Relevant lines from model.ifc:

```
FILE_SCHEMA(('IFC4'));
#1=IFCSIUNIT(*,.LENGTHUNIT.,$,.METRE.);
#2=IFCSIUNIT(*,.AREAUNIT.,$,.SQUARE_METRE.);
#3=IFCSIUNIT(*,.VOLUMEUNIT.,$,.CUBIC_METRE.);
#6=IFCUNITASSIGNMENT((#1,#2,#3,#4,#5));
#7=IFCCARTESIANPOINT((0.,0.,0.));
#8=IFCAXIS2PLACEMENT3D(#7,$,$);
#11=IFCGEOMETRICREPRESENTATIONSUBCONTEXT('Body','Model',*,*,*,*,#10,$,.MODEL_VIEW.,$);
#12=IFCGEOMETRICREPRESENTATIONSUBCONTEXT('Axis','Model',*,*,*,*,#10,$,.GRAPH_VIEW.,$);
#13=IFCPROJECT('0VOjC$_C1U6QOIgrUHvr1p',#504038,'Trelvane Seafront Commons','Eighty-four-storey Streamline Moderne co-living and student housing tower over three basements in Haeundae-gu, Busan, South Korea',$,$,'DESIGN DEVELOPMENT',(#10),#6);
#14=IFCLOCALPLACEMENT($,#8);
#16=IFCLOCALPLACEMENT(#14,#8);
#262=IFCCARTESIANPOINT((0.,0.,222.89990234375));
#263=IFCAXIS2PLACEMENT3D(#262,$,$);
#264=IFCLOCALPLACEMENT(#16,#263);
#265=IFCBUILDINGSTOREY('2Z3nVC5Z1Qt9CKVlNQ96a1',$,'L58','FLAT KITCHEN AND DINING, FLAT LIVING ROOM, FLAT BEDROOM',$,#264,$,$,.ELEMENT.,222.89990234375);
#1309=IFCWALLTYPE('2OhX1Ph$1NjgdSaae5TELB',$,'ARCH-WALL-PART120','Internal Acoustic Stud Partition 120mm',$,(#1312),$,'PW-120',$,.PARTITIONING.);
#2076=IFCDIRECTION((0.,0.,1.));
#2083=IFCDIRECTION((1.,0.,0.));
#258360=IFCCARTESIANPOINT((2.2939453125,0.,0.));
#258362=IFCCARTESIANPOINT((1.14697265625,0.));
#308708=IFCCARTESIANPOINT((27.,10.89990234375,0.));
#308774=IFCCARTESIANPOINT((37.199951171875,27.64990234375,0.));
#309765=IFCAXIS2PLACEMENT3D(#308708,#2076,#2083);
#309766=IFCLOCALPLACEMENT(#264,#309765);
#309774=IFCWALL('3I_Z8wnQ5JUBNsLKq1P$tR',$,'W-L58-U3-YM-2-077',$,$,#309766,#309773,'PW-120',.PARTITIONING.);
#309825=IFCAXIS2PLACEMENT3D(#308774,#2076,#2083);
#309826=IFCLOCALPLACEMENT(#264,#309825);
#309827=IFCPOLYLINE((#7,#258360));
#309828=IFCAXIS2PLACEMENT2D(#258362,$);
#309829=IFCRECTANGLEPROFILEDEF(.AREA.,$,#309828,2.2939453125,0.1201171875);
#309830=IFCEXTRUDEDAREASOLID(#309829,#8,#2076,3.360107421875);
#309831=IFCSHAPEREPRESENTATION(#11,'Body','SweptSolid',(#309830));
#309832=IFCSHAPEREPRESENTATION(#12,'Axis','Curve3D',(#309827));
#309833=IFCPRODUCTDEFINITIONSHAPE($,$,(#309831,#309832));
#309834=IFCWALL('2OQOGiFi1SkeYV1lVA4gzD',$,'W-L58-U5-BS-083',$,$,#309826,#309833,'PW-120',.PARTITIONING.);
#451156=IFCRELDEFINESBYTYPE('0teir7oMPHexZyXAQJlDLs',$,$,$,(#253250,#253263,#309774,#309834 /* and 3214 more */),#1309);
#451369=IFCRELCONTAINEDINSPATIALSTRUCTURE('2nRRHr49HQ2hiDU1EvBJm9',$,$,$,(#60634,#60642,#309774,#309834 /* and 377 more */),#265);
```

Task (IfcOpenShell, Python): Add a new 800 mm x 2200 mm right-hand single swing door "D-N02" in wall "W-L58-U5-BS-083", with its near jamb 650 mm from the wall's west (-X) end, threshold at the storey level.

```python
import numpy as np
import ifcopenshell
import ifcopenshell.api.feature
import ifcopenshell.api.geometry
import ifcopenshell.api.root
import ifcopenshell.api.spatial
import ifcopenshell.geom
import ifcopenshell.util.element
import ifcopenshell.util.placement
import ifcopenshell.util.representation
import ifcopenshell.util.shape
import ifcopenshell.util.unit

model = ifcopenshell.open("model.ifc")
unit_scale = ifcopenshell.util.unit.calculate_unit_scale(model)
settings = ifcopenshell.geom.settings()


def volume(element):
    """Net volume in cubic metres, openings subtracted."""
    shape = ifcopenshell.geom.create_shape(settings, element)
    return ifcopenshell.util.shape.get_volume(shape.geometry)


wall = model.by_id(309834)
storey = ifcopenshell.util.element.get_container(wall, ifc_class="IfcBuildingStorey")
context = ifcopenshell.util.representation.get_context(model, "Model", "Body", "MODEL_VIEW")
before = volume(wall)

width, height, from_end, sill = 0.8, 2.2, 0.65, 0.0  # metres

# The wall runs along its own X axis, and the end named is its -X end.
wall_shape = ifcopenshell.geom.create_shape(settings, wall)
x, y, z = ifcopenshell.util.shape.get_vertices(wall_shape.geometry).T
start = x.min() + from_end
face, thickness = float(y.min()), float(y.max() - y.min())
wall_matrix = ifcopenshell.util.placement.get_local_placement(wall.ObjectPlacement)
level = ifcopenshell.util.placement.get_local_placement(storey.ObjectPlacement)[2, 3]


def in_wall(x, y):
    """Placement at x, y metres in the wall's axes, at sill height."""
    matrix = wall_matrix.copy()
    matrix[:, 3] = wall_matrix @ np.array([x / unit_scale, y / unit_scale, 0.0, 1.0])
    matrix[2, 3] = level + sill / unit_scale
    return matrix


# Opening: a box that overshoots both wall faces by 50 mm.
opening = ifcopenshell.api.root.create_entity(model, ifc_class="IfcOpeningElement", predefined_type="OPENING")
box = ifcopenshell.api.geometry.add_wall_representation(
    model, context=context, length=width, height=height, thickness=thickness + 0.1
)
ifcopenshell.api.geometry.assign_representation(model, product=opening, representation=box)
ifcopenshell.api.geometry.edit_object_placement(model, product=opening, matrix=in_wall(start, face - 0.05), is_si=False)
ifcopenshell.api.feature.add_feature(model, feature=opening, element=wall)

door = ifcopenshell.api.root.create_entity(model, ifc_class="IfcDoor", name="D-N02", predefined_type="DOOR")
door.OverallWidth, door.OverallHeight = width / unit_scale, height / unit_scale
door.OperationType = "SINGLE_SWING_RIGHT"
body = ifcopenshell.api.geometry.add_door_representation(
    model,
    context=context,
    overall_width=door.OverallWidth,
    overall_height=door.OverallHeight,
    operation_type="SINGLE_SWING_RIGHT",
    lining_properties={"LiningDepth": thickness / unit_scale, "ThresholdDepth": thickness / unit_scale},
)
ifcopenshell.api.geometry.assign_representation(model, product=door, representation=body)
ifcopenshell.api.spatial.assign_container(model, products=[door], relating_structure=storey)
ifcopenshell.api.feature.add_filling(model, opening=opening, element=door)

# The lining spans the wall, so the door starts at the wall face.
ifcopenshell.api.geometry.edit_object_placement(model, product=door, matrix=in_wall(start, face), is_si=False)

after = volume(wall)

print(f"wall volume {before:.3f} -> {after:.3f} m3")

model.write("model_v2.ifc")
```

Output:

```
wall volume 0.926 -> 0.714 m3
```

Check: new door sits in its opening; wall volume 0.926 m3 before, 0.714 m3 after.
